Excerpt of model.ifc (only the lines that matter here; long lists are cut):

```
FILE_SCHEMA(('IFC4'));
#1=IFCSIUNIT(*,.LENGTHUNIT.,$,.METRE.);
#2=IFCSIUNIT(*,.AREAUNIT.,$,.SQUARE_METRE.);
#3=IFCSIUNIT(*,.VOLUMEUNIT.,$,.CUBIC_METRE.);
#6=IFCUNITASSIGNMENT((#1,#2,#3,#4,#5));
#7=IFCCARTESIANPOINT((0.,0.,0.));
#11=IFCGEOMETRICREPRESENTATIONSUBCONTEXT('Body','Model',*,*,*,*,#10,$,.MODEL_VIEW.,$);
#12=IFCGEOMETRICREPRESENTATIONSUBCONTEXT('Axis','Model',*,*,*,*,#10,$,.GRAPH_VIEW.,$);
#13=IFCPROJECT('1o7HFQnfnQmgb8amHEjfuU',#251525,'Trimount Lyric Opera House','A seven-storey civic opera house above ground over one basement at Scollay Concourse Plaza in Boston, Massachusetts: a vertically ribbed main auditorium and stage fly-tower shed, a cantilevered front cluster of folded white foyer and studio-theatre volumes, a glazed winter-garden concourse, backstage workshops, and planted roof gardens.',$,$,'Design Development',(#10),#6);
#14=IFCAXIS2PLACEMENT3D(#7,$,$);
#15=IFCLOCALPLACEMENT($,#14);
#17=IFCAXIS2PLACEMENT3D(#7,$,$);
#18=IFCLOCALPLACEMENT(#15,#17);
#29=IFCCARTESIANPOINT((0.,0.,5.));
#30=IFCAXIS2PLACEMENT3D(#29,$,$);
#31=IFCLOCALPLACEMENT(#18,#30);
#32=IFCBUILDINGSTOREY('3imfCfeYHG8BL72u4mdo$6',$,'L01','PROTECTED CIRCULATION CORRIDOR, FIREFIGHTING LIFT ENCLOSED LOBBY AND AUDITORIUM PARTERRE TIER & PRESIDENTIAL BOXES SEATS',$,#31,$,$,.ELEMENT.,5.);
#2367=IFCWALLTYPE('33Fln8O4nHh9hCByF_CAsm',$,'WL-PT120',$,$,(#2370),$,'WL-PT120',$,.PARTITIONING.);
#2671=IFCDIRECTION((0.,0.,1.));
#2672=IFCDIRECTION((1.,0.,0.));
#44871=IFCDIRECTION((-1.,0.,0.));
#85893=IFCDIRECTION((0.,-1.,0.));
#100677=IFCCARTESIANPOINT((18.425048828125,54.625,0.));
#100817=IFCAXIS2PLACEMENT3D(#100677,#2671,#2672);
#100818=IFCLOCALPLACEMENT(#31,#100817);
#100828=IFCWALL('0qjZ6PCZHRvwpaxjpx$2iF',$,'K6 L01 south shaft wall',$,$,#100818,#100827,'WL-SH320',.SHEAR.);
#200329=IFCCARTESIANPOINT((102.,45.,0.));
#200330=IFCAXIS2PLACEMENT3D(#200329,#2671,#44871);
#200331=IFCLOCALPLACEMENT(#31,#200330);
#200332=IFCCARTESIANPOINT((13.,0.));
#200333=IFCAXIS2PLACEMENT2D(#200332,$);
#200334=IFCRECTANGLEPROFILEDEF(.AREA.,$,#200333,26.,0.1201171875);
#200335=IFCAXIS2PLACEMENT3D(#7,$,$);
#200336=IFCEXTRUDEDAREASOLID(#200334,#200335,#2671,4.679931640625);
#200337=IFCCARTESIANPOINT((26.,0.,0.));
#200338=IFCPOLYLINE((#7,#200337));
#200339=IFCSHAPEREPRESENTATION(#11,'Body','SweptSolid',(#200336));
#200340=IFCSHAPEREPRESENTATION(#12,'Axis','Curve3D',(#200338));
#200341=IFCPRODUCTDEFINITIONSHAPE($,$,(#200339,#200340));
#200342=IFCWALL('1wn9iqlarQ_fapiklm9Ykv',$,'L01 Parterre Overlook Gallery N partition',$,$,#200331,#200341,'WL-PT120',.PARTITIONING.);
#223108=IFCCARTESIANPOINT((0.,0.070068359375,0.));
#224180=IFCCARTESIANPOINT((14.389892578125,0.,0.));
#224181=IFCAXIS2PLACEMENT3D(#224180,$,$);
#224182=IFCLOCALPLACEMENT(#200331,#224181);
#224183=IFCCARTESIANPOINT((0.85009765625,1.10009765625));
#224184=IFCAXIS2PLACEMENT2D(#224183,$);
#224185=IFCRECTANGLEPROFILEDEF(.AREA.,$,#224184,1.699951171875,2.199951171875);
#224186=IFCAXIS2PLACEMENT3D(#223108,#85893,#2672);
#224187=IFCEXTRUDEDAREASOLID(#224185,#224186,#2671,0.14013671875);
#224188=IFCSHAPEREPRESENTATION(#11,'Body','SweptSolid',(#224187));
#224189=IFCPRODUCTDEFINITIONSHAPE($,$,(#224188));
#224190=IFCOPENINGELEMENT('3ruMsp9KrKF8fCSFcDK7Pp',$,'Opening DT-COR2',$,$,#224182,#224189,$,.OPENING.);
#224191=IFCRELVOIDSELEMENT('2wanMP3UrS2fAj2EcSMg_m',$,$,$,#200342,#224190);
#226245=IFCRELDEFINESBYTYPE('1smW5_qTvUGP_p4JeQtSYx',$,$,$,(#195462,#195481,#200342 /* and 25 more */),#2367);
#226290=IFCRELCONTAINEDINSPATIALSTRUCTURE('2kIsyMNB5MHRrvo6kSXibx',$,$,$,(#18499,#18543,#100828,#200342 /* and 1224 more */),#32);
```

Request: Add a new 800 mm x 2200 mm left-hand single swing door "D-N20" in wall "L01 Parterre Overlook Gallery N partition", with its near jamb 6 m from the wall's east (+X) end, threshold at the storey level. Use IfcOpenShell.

```python
import numpy as np
import ifcopenshell
import ifcopenshell.api.feature
import ifcopenshell.api.geometry
import ifcopenshell.api.root
import ifcopenshell.api.spatial
import ifcopenshell.geom
import ifcopenshell.util.element
import ifcopenshell.util.placement
import ifcopenshell.util.representation
import ifcopenshell.util.shape
import ifcopenshell.util.unit

model = ifcopenshell.open("model.ifc")
unit_scale = ifcopenshell.util.unit.calculate_unit_scale(model)
settings = ifcopenshell.geom.settings()


def volume(element):
    """Net volume in cubic metres, openings subtracted."""
    shape = ifcopenshell.geom.create_shape(settings, element)
    return ifcopenshell.util.shape.get_volume(shape.geometry)


wall = model.by_guid("1wn9iqlarQ_fapiklm9Ykv")
storey = ifcopenshell.util.element.get_container(wall, ifc_class="IfcBuildingStorey")
context = ifcopenshell.util.representation.get_context(model, "Model", "Body", "MODEL_VIEW")
before = volume(wall)

width, height, from_end, sill = 0.8, 2.2, 6, 0.0  # metres

# The wall runs along its own X axis, and the end named is its -X end.
wall_shape = ifcopenshell.geom.create_shape(settings, wall)
x, y, z = ifcopenshell.util.shape.get_vertices(wall_shape.geometry).T
start = x.min() + from_end
face, thickness = float(y.min()), float(y.max() - y.min())
wall_matrix = ifcopenshell.util.placement.get_local_placement(wall.ObjectPlacement)
level = ifcopenshell.util.placement.get_local_placement(storey.ObjectPlacement)[2, 3]


def in_wall(x, y):
    """Placement at x, y metres in the wall's axes, at sill height."""
    matrix = wall_matrix.copy()
    matrix[:, 3] = wall_matrix @ np.array([x / unit_scale, y / unit_scale, 0.0, 1.0])
    matrix[2, 3] = level + sill / unit_scale
    return matrix


# Opening: a box that overshoots both wall faces by 50 mm.
opening = ifcopenshell.api.root.create_entity(model, ifc_class="IfcOpeningElement", predefined_type="OPENING")
box = ifcopenshell.api.geometry.add_wall_representation(
    model, context=context, length=width, height=height, thickness=thickness + 0.1
)
ifcopenshell.api.geometry.assign_representation(model, product=opening, representation=box)
ifcopenshell.api.geometry.edit_object_placement(model, product=opening, matrix=in_wall(start, face - 0.05), is_si=False)
ifcopenshell.api.feature.add_feature(model, feature=opening, element=wall)

door = ifcopenshell.api.root.create_entity(model, ifc_class="IfcDoor", name="D-N20", predefined_type="DOOR")
door.OverallWidth, door.OverallHeight = width / unit_scale, height / unit_scale
door.OperationType = "SINGLE_SWING_LEFT"
body = ifcopenshell.api.geometry.add_door_representation(
    model,
    context=context,
    overall_width=door.OverallWidth,
    overall_height=door.OverallHeight,
    operation_type="SINGLE_SWING_LEFT",
    lining_properties={"LiningDepth": thickness / unit_scale, "ThresholdDepth": thickness / unit_scale},
)
ifcopenshell.api.geometry.assign_representation(model, product=door, representation=body)
ifcopenshell.api.spatial.assign_container(model, products=[door], relating_structure=storey)
ifcopenshell.api.feature.add_filling(model, opening=opening, element=door)

# The lining spans the wall, so the door starts at the wall face.
ifcopenshell.api.geometry.edit_object_placement(model, product=door, matrix=in_wall(start, face), is_si=False)

after = volume(wall)

print(f"wall volume {before:.3f} -> {after:.3f} m3")

model.write("model_edited.ifc")
```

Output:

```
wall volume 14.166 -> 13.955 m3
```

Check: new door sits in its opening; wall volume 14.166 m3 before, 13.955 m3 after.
